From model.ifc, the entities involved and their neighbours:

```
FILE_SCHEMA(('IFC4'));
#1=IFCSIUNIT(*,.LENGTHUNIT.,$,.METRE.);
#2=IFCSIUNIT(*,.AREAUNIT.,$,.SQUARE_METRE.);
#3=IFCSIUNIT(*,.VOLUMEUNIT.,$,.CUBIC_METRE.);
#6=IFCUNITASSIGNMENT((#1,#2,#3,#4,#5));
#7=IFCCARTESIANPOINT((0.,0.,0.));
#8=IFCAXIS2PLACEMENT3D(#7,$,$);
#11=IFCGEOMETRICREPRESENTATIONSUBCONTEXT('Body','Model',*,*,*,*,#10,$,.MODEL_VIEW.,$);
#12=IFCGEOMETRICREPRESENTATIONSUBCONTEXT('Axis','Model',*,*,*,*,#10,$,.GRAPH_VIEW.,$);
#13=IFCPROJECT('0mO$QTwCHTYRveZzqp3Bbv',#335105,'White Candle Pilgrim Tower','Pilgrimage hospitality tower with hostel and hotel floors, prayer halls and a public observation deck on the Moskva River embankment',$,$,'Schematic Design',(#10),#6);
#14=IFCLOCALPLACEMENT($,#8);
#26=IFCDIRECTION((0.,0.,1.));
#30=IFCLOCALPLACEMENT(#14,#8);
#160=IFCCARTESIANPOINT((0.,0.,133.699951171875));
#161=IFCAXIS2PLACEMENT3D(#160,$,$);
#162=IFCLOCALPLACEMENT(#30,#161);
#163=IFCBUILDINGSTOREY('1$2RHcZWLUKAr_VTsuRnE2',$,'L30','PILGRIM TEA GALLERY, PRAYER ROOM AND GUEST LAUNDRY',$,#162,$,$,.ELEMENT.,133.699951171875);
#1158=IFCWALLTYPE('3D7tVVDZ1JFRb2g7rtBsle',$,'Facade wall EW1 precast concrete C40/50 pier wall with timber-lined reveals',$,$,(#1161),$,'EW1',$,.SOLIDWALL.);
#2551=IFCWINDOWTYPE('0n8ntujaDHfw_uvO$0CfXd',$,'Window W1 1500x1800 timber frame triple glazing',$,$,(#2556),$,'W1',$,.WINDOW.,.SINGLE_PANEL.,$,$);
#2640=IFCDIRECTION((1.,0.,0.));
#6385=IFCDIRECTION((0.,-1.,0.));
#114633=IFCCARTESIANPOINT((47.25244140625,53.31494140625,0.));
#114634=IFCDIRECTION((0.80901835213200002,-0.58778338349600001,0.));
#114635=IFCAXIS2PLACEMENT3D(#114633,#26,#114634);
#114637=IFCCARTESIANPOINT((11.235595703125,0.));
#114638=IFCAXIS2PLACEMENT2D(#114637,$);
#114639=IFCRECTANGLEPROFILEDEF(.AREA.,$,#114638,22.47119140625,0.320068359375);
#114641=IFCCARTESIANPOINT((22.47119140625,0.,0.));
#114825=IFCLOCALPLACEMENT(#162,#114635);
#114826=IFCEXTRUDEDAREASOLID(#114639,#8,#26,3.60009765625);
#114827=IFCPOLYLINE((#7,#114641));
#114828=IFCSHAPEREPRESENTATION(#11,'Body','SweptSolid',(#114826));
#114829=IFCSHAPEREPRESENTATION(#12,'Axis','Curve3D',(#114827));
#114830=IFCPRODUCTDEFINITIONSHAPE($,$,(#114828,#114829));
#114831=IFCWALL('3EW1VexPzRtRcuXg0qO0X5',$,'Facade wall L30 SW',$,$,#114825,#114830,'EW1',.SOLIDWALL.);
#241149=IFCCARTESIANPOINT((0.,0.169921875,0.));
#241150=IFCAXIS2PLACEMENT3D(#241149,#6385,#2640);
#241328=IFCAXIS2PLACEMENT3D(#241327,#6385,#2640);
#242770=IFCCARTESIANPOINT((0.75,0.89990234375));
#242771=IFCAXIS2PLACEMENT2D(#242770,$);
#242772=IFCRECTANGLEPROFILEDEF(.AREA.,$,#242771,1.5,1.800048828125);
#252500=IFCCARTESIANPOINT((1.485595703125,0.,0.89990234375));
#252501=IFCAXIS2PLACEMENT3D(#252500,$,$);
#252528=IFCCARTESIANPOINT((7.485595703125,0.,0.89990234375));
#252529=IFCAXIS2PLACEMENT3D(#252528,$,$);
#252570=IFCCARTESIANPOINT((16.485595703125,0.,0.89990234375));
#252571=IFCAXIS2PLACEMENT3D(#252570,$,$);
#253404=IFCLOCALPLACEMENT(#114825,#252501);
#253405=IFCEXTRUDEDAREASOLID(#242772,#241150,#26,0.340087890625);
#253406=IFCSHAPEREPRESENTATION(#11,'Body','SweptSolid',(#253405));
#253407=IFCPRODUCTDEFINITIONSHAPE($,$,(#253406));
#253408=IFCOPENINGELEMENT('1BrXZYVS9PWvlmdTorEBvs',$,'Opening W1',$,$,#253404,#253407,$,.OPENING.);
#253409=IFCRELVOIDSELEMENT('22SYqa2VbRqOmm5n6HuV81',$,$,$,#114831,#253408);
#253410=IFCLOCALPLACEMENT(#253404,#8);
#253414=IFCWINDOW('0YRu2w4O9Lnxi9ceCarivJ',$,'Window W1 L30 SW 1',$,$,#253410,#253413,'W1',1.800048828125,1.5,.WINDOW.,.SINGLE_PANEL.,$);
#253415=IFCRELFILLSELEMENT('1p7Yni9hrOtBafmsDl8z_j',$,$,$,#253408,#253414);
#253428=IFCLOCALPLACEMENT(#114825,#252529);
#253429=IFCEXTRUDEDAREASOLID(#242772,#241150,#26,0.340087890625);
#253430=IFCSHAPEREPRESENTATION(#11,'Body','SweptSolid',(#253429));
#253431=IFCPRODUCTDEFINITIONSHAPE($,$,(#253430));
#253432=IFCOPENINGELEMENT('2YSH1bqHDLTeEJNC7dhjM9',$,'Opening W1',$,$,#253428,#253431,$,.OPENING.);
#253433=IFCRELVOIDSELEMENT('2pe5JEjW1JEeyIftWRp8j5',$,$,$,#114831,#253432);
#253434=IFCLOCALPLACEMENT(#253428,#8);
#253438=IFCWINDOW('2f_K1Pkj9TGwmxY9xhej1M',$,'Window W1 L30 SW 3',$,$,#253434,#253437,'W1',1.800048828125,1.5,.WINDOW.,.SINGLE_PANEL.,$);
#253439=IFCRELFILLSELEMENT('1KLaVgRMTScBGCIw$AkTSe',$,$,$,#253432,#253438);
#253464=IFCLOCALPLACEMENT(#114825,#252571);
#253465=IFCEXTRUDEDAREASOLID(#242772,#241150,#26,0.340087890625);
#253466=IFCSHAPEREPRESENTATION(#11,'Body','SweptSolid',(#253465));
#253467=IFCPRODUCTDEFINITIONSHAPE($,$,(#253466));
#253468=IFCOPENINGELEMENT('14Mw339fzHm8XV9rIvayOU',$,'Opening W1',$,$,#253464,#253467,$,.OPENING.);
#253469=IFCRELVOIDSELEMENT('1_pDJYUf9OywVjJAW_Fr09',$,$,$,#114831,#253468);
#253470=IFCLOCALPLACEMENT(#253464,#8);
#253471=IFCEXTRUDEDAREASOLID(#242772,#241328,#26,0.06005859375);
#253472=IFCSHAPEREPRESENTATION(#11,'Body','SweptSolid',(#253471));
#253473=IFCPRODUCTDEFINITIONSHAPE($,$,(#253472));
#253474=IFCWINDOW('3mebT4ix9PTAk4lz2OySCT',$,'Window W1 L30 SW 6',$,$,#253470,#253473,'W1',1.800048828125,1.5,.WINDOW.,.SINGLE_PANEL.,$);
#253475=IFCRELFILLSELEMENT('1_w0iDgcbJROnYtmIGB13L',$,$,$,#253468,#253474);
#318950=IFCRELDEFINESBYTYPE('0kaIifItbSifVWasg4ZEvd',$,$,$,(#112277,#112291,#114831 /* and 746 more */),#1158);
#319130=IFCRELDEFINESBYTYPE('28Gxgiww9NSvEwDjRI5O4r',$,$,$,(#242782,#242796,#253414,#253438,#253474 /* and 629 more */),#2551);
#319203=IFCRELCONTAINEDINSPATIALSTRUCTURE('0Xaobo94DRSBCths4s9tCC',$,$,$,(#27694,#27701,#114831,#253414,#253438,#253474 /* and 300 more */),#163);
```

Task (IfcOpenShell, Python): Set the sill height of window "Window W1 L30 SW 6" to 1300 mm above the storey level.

```python
import numpy as np
import ifcopenshell
import ifcopenshell.api.geometry
import ifcopenshell.geom
import ifcopenshell.util.element
import ifcopenshell.util.placement
import ifcopenshell.util.shape
import ifcopenshell.util.unit

model = ifcopenshell.open("model.ifc")
unit_scale = ifcopenshell.util.unit.calculate_unit_scale(model)

window = model.by_guid("3mebT4ix9PTAk4lz2OySCT")
opening = window.FillsVoids[0].RelatingOpeningElement
storey = ifcopenshell.util.element.get_container(window, ifc_class="IfcBuildingStorey")
level = ifcopenshell.util.placement.get_local_placement(storey.ObjectPlacement)[2, 3]

# The opening's origin need not be at the sill, so measure its lowest point.
shape = ifcopenshell.geom.create_shape(ifcopenshell.geom.settings(), opening)
bottom = ifcopenshell.util.shape.get_shape_bottom_elevation(shape, shape.geometry) / unit_scale
dz = level + 1.3 / unit_scale - bottom

shift = np.array([0.0, 0.0, dz])
# The window is placed relative to its opening, so it follows when the opening moves.
matrix = ifcopenshell.util.placement.get_local_placement(opening.ObjectPlacement)
matrix[:3, 3] += shift
ifcopenshell.api.geometry.edit_object_placement(
    model, product=opening, matrix=matrix, is_si=False, should_transform_children=True
)

print(f"moved by {dz * unit_scale:+.3f} m")

model.write("model-out.ifc")
```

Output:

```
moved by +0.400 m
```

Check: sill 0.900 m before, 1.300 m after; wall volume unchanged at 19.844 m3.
